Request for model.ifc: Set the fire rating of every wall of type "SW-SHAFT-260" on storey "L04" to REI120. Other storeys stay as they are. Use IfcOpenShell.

First a look at what the model holds.

```python
import ifcopenshell
import ifcopenshell.util.element

model = ifcopenshell.open("model.ifc")
print(model.schema)
storey = next(s for s in model.by_type("IfcBuildingStorey") if s.Name == "L04")
walls = [e for e in ifcopenshell.util.element.get_decomposition(storey) if e.is_a("IfcWall")]
seen = {}
for e in walls:
    element_type = ifcopenshell.util.element.get_type(e)
    key = (element_type.Name if element_type != e and element_type else None, ifcopenshell.util.element.get_pset(e, "Pset_WallCommon", "FireRating"))
    seen[key] = seen.get(key, 0) + 1
for (name, value), count in sorted(seen.items(), key=str):
    print(count, "x", name, "|", value)
```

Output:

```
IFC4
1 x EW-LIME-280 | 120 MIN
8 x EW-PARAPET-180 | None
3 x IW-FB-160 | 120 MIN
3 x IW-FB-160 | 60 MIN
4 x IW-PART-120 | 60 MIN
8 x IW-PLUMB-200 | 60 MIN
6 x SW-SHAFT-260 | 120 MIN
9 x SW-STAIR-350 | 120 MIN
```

```python
import ifcopenshell
import ifcopenshell.api.pset
import ifcopenshell.util.element

model = ifcopenshell.open("model.ifc")

storey = next(s for s in model.by_type("IfcBuildingStorey") if s.Name == "L04")
walls = [e for e in ifcopenshell.util.element.get_decomposition(storey) if e.is_a("IfcWall")]

count = 0
for e in walls:
    element_type = ifcopenshell.util.element.get_type(e)
    if element_type in (None, e) or element_type.Name != "SW-SHAFT-260":
        continue
    # add_pset returns the element's existing set when there is one.
    pset = ifcopenshell.api.pset.add_pset(model, product=e, name="Pset_WallCommon")
    ifcopenshell.api.pset.edit_pset(model, pset=pset, properties={"FireRating": "REI120"})
    count += 1

print(count, "walls updated")

model.write("model_edited.ifc")
```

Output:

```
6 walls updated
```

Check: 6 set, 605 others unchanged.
